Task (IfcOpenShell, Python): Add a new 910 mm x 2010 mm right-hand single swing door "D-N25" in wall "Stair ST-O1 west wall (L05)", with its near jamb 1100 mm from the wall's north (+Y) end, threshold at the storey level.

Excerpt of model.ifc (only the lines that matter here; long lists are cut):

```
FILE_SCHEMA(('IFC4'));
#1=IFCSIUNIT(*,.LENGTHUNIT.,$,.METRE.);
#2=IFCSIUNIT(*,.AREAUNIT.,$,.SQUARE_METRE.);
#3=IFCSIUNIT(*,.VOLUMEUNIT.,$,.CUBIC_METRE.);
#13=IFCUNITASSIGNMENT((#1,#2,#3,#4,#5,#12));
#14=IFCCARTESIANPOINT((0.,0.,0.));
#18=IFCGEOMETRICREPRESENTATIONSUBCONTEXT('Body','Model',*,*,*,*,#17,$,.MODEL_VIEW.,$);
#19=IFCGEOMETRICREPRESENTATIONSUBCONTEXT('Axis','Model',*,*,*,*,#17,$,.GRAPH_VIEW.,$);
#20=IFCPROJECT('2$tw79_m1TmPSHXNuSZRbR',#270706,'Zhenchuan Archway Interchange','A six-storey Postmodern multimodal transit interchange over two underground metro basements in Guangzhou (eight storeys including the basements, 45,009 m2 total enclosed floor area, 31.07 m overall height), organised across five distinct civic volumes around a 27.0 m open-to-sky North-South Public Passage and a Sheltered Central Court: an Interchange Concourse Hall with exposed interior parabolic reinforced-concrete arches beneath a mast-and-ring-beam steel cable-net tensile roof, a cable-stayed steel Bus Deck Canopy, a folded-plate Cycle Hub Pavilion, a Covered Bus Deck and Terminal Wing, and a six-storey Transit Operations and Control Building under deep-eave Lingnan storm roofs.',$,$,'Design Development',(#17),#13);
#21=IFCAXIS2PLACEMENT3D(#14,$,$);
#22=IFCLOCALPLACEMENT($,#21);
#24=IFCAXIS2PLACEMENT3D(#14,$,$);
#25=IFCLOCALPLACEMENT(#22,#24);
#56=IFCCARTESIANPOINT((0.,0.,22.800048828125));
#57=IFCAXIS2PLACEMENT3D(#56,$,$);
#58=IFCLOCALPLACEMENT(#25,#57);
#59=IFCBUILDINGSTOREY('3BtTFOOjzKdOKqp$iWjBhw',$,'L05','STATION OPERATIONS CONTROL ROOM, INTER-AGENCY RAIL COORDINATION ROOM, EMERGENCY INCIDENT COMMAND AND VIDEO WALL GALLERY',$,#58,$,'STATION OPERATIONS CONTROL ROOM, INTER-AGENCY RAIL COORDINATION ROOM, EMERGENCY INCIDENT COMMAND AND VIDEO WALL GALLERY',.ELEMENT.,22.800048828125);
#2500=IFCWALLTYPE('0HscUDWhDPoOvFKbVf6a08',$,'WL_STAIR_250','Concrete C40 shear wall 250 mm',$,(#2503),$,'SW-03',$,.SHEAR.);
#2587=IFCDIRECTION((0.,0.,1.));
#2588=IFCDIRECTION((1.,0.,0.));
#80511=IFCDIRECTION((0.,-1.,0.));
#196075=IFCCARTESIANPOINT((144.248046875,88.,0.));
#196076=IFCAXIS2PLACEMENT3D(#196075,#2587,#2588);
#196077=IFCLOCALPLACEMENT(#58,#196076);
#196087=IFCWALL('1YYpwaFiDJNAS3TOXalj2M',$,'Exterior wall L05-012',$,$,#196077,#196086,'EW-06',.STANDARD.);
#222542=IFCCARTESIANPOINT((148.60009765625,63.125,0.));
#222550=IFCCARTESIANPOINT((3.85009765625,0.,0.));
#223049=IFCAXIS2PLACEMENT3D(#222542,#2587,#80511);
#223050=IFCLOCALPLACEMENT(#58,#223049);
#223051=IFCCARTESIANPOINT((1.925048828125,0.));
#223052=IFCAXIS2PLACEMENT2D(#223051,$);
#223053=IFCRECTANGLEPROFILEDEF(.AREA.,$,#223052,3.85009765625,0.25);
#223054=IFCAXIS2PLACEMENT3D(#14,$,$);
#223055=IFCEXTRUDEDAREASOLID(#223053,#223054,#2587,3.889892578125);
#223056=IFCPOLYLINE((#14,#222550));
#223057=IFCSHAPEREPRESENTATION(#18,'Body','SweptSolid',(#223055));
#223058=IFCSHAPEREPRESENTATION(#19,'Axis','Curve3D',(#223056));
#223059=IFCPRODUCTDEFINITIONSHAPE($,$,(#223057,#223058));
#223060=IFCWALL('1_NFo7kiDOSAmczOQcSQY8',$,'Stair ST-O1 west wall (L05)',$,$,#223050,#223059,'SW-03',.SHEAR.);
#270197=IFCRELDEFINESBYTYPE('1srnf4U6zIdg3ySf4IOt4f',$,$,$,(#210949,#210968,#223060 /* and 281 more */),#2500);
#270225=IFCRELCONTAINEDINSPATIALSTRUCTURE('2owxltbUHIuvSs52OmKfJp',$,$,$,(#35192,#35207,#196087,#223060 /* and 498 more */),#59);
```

```python
import numpy as np
import ifcopenshell
import ifcopenshell.api.feature
import ifcopenshell.api.geometry
import ifcopenshell.api.root
import ifcopenshell.api.spatial
import ifcopenshell.geom
import ifcopenshell.util.element
import ifcopenshell.util.placement
import ifcopenshell.util.representation
import ifcopenshell.util.shape
import ifcopenshell.util.unit

model = ifcopenshell.open("model.ifc")
unit_scale = ifcopenshell.util.unit.calculate_unit_scale(model)
settings = ifcopenshell.geom.settings()


def volume(element):
    """Net volume in cubic metres, openings subtracted."""
    shape = ifcopenshell.geom.create_shape(settings, element)
    return ifcopenshell.util.shape.get_volume(shape.geometry)


wall = model.by_id(223060)
storey = ifcopenshell.util.element.get_container(wall, ifc_class="IfcBuildingStorey")
context = ifcopenshell.util.representation.get_context(model, "Model", "Body", "MODEL_VIEW")
before = volume(wall)

width, height, from_end, sill = 0.91, 2.01, 1.1, 0.0  # metres

# The wall runs along its own X axis, and the end named is its -X end.
wall_shape = ifcopenshell.geom.create_shape(settings, wall)
x, y, z = ifcopenshell.util.shape.get_vertices(wall_shape.geometry).T
start = x.min() + from_end
face, thickness = float(y.min()), float(y.max() - y.min())
wall_matrix = ifcopenshell.util.placement.get_local_placement(wall.ObjectPlacement)
level = ifcopenshell.util.placement.get_local_placement(storey.ObjectPlacement)[2, 3]


def in_wall(x, y):
    """Placement at x, y metres in the wall's axes, at sill height."""
    matrix = wall_matrix.copy()
    matrix[:, 3] = wall_matrix @ np.array([x / unit_scale, y / unit_scale, 0.0, 1.0])
    matrix[2, 3] = level + sill / unit_scale
    return matrix


# Opening: a box that overshoots both wall faces by 50 mm.
opening = ifcopenshell.api.root.create_entity(model, ifc_class="IfcOpeningElement", predefined_type="OPENING")
box = ifcopenshell.api.geometry.add_wall_representation(
    model, context=context, length=width, height=height, thickness=thickness + 0.1
)
ifcopenshell.api.geometry.assign_representation(model, product=opening, representation=box)
ifcopenshell.api.geometry.edit_object_placement(model, product=opening, matrix=in_wall(start, face - 0.05), is_si=False)
ifcopenshell.api.feature.add_feature(model, feature=opening, element=wall)

door = ifcopenshell.api.root.create_entity(model, ifc_class="IfcDoor", name="D-N25", predefined_type="DOOR")
door.OverallWidth, door.OverallHeight = width / unit_scale, height / unit_scale
door.OperationType = "SINGLE_SWING_RIGHT"
body = ifcopenshell.api.geometry.add_door_representation(
    model,
    context=context,
    overall_width=door.OverallWidth,
    overall_height=door.OverallHeight,
    operation_type="SINGLE_SWING_RIGHT",
    lining_properties={"LiningDepth": thickness / unit_scale, "ThresholdDepth": thickness / unit_scale},
)
ifcopenshell.api.geometry.assign_representation(model, product=door, representation=body)
ifcopenshell.api.spatial.assign_container(model, products=[door], relating_structure=storey)
ifcopenshell.api.feature.add_filling(model, opening=opening, element=door)

# The lining spans the wall, so the door starts at the wall face.
ifcopenshell.api.geometry.edit_object_placement(model, product=door, matrix=in_wall(start, face), is_si=False)

after = volume(wall)

print(f"wall volume {before:.3f} -> {after:.3f} m3")

model.write("model_rev.ifc")
```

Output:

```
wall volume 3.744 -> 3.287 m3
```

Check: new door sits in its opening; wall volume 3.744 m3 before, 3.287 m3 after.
